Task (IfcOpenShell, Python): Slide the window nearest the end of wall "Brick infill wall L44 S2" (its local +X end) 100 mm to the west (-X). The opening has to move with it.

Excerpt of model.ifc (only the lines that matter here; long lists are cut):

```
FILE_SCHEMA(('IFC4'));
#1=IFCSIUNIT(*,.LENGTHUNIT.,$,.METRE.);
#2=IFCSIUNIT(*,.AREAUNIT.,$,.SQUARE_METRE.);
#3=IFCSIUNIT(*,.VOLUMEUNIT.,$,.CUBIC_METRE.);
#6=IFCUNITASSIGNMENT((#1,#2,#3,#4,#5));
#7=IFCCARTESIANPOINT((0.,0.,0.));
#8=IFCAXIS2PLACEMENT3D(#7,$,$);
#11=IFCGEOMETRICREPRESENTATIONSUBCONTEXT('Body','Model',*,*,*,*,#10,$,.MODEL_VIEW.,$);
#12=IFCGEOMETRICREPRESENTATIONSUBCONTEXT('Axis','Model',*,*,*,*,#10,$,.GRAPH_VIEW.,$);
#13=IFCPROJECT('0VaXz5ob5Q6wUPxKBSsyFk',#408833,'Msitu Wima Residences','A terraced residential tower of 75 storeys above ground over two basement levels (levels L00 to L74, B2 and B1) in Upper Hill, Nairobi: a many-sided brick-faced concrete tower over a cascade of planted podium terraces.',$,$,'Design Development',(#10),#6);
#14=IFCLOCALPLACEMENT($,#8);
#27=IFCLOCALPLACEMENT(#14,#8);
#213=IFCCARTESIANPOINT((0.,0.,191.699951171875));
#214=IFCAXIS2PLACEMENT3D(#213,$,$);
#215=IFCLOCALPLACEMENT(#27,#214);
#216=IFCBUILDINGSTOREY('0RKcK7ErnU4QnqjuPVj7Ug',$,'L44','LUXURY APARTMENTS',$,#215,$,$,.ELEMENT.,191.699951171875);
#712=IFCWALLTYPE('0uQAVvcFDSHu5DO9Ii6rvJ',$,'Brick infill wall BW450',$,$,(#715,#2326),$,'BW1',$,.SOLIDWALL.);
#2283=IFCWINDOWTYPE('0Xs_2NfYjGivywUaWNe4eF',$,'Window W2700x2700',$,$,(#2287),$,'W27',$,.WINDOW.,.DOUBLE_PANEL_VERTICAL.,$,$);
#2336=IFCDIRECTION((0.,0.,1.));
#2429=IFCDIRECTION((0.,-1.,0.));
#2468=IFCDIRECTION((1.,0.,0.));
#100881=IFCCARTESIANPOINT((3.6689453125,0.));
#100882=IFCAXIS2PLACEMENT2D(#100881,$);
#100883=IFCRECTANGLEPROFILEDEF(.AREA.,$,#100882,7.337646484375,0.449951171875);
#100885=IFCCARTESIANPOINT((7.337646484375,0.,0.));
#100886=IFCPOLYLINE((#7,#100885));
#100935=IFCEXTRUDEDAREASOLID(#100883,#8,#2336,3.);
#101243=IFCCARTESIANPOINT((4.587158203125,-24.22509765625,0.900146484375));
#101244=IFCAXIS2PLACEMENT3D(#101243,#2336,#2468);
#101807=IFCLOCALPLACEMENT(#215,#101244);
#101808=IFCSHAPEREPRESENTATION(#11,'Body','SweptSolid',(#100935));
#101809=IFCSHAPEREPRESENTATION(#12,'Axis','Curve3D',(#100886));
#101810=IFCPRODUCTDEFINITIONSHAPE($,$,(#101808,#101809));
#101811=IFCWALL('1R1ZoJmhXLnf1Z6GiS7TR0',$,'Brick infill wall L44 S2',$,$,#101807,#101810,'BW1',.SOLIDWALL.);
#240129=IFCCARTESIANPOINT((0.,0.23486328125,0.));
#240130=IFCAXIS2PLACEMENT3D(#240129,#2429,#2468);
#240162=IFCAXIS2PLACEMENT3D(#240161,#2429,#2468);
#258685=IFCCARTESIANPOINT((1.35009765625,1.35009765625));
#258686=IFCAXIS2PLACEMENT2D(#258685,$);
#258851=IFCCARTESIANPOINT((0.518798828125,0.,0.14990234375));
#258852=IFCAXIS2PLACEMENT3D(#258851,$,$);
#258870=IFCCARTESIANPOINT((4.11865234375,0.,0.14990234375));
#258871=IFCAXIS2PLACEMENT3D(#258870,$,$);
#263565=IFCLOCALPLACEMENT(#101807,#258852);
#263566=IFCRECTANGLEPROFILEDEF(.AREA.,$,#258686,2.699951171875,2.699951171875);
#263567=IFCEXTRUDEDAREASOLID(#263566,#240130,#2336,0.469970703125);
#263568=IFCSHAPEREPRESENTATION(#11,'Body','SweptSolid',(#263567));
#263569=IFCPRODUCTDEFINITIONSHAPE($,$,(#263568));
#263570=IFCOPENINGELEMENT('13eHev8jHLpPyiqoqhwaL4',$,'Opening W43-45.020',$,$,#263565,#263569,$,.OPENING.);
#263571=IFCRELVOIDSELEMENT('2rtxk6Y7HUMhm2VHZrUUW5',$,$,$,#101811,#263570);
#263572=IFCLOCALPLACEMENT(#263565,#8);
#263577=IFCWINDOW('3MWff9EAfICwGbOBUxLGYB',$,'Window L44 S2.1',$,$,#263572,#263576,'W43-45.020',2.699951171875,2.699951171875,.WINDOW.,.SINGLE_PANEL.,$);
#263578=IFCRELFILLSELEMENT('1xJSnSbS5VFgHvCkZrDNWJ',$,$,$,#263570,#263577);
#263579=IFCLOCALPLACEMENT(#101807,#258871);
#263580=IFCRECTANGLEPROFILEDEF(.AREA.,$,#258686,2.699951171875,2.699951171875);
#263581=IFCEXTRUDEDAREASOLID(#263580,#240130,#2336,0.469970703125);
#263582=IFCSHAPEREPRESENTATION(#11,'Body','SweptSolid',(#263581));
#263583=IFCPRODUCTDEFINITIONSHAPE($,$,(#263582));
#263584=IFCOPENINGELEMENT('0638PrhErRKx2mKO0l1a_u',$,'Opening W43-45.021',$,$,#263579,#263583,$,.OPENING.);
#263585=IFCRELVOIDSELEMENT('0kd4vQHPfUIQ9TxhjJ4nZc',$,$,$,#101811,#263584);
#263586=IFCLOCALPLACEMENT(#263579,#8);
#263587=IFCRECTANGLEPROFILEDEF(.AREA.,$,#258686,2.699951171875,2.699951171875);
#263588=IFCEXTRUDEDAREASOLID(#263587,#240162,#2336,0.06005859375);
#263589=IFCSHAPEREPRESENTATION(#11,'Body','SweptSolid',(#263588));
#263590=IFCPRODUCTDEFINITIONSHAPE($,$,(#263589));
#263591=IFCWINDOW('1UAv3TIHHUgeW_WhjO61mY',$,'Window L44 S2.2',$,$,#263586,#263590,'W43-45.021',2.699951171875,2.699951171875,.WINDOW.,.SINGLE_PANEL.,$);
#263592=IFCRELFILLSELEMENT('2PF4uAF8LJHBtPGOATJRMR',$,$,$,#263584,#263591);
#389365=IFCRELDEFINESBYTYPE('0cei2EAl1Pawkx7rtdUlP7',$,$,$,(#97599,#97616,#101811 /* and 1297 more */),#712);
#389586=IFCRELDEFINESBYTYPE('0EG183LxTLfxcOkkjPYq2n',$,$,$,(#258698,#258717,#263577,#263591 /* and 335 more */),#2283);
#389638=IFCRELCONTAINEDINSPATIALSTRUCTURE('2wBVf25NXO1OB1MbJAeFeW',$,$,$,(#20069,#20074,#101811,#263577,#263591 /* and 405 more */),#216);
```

```python
import ifcopenshell
import ifcopenshell.api.geometry
import ifcopenshell.util.placement

model = ifcopenshell.open("model.ifc")

window = model.by_id(263591)
opening = window.FillsVoids[0].RelatingOpeningElement
wall = opening.VoidsElements[0].RelatingBuildingElement

wall_matrix = ifcopenshell.util.placement.get_local_placement(wall.ObjectPlacement)
shift = wall_matrix[:3, 0] * -0.1
before = ifcopenshell.util.placement.get_local_placement(window.ObjectPlacement)[:3, 3].copy()

# The window is placed relative to its opening, so it follows when the opening moves.
matrix = ifcopenshell.util.placement.get_local_placement(opening.ObjectPlacement)
matrix[:3, 3] += shift
ifcopenshell.api.geometry.edit_object_placement(
    model, product=opening, matrix=matrix, is_si=False, should_transform_children=True
)

after = ifcopenshell.util.placement.get_local_placement(window.ObjectPlacement)[:3, 3]
print("window moved by", (after - before).round(3) + 0.0)

model.write("model-out.ifc")
```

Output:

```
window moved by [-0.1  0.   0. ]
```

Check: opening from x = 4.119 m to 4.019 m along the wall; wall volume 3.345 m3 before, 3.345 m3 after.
